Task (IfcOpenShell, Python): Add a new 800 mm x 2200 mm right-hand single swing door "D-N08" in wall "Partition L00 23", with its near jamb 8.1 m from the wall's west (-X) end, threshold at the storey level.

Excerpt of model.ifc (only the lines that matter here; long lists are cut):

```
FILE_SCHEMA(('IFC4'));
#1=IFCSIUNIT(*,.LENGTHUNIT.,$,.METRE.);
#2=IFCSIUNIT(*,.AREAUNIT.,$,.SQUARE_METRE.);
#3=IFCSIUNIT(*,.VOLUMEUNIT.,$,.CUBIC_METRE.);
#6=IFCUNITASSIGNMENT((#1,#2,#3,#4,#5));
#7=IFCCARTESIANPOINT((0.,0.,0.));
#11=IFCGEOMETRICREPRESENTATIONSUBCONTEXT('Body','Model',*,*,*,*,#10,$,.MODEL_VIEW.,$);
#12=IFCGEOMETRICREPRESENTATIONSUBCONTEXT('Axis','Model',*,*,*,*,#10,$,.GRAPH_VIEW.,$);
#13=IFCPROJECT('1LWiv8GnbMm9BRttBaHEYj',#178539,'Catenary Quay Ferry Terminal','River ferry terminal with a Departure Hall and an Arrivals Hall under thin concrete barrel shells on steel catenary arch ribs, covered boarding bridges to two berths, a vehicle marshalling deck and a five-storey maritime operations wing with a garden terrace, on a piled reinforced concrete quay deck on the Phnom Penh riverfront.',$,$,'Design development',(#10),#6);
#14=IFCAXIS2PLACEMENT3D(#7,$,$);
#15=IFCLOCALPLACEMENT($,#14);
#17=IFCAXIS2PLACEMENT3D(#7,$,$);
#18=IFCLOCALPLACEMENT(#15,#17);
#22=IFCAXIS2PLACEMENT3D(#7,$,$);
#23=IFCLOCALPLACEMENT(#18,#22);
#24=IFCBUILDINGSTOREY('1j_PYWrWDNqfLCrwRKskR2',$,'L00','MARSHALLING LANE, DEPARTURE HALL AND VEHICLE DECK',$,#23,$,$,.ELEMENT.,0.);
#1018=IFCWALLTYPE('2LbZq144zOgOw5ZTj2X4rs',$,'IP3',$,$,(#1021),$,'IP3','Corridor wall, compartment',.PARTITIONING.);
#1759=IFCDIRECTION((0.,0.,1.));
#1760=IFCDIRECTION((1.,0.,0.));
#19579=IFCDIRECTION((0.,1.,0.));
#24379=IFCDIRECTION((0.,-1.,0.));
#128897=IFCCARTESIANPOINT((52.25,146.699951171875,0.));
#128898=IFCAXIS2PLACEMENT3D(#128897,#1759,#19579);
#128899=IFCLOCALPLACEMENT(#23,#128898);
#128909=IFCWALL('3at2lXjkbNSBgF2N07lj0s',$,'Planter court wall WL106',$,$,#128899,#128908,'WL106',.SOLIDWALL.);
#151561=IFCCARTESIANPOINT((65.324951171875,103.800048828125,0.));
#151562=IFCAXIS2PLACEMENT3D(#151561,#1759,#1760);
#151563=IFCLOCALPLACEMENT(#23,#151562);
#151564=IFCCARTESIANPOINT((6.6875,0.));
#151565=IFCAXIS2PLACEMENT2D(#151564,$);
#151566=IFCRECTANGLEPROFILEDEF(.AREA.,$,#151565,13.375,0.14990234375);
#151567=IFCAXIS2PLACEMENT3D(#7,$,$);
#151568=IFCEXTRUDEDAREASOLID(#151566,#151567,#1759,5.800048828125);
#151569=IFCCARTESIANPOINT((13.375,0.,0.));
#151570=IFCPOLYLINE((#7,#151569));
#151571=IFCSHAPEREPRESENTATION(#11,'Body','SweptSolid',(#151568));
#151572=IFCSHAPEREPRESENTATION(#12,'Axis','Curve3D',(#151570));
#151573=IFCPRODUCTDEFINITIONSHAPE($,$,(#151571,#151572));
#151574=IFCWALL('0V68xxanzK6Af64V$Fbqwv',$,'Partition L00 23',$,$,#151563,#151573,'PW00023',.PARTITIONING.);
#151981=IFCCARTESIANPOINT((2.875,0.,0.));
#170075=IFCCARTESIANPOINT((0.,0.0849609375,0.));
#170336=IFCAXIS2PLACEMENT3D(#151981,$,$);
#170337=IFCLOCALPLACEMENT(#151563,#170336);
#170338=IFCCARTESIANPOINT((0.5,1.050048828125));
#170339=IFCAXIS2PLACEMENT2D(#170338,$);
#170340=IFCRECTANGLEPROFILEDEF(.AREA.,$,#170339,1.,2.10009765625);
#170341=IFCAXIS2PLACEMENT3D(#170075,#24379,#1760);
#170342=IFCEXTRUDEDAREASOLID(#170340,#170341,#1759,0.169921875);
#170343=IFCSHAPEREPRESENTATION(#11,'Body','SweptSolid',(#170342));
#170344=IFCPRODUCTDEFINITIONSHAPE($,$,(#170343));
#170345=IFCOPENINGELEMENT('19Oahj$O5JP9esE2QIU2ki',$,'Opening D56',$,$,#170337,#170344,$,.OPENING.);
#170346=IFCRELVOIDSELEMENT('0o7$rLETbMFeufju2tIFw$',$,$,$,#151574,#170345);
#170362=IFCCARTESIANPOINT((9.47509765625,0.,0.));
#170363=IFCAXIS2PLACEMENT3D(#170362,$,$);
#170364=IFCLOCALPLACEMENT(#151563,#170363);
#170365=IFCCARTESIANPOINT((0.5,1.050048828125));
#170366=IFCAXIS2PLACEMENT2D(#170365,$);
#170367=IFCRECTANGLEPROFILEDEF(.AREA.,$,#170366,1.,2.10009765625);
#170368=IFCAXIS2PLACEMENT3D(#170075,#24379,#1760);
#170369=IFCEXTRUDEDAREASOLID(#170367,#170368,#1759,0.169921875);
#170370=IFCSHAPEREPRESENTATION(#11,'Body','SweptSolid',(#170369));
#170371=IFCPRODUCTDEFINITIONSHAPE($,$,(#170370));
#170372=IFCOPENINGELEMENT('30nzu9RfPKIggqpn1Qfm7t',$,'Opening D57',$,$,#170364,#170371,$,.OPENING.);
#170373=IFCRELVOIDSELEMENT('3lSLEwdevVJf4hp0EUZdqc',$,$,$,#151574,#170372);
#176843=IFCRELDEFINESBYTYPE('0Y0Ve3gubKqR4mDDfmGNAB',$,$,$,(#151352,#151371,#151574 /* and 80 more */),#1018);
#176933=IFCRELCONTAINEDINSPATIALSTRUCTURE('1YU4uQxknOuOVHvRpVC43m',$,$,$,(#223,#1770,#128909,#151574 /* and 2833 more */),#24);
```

```python
import numpy as np
import ifcopenshell
import ifcopenshell.api.feature
import ifcopenshell.api.geometry
import ifcopenshell.api.root
import ifcopenshell.api.spatial
import ifcopenshell.geom
import ifcopenshell.util.element
import ifcopenshell.util.placement
import ifcopenshell.util.representation
import ifcopenshell.util.shape
import ifcopenshell.util.unit

model = ifcopenshell.open("model.ifc")
unit_scale = ifcopenshell.util.unit.calculate_unit_scale(model)
settings = ifcopenshell.geom.settings()


def volume(element):
    """Net volume in cubic metres, openings subtracted."""
    shape = ifcopenshell.geom.create_shape(settings, element)
    return ifcopenshell.util.shape.get_volume(shape.geometry)


wall = model.by_guid("0V68xxanzK6Af64V$Fbqwv")
storey = ifcopenshell.util.element.get_container(wall, ifc_class="IfcBuildingStorey")
context = ifcopenshell.util.representation.get_context(model, "Model", "Body", "MODEL_VIEW")
before = volume(wall)

width, height, from_end, sill = 0.8, 2.2, 8.1, 0.0  # metres

# The wall runs along its own X axis, and the end named is its -X end.
wall_shape = ifcopenshell.geom.create_shape(settings, wall)
x, y, z = ifcopenshell.util.shape.get_vertices(wall_shape.geometry).T
start = x.min() + from_end
face, thickness = float(y.min()), float(y.max() - y.min())
wall_matrix = ifcopenshell.util.placement.get_local_placement(wall.ObjectPlacement)
level = ifcopenshell.util.placement.get_local_placement(storey.ObjectPlacement)[2, 3]


def in_wall(x, y):
    """Placement at x, y metres in the wall's axes, at sill height."""
    matrix = wall_matrix.copy()
    matrix[:, 3] = wall_matrix @ np.array([x / unit_scale, y / unit_scale, 0.0, 1.0])
    matrix[2, 3] = level + sill / unit_scale
    return matrix


# Opening: a box that overshoots both wall faces by 50 mm.
opening = ifcopenshell.api.root.create_entity(model, ifc_class="IfcOpeningElement", predefined_type="OPENING")
box = ifcopenshell.api.geometry.add_wall_representation(
    model, context=context, length=width, height=height, thickness=thickness + 0.1
)
ifcopenshell.api.geometry.assign_representation(model, product=opening, representation=box)
ifcopenshell.api.geometry.edit_object_placement(model, product=opening, matrix=in_wall(start, face - 0.05), is_si=False)
ifcopenshell.api.feature.add_feature(model, feature=opening, element=wall)

door = ifcopenshell.api.root.create_entity(model, ifc_class="IfcDoor", name="D-N08", predefined_type="DOOR")
door.OverallWidth, door.OverallHeight = width / unit_scale, height / unit_scale
door.OperationType = "SINGLE_SWING_RIGHT"
body = ifcopenshell.api.geometry.add_door_representation(
    model,
    context=context,
    overall_width=door.OverallWidth,
    overall_height=door.OverallHeight,
    operation_type="SINGLE_SWING_RIGHT",
    lining_properties={"LiningDepth": thickness / unit_scale, "ThresholdDepth": thickness / unit_scale},
)
ifcopenshell.api.geometry.assign_representation(model, product=door, representation=body)
ifcopenshell.api.spatial.assign_container(model, products=[door], relating_structure=storey)
ifcopenshell.api.feature.add_filling(model, opening=opening, element=door)

# The lining spans the wall, so the door starts at the wall face.
ifcopenshell.api.geometry.edit_object_placement(model, product=door, matrix=in_wall(start, face), is_si=False)

after = volume(wall)

print(f"wall volume {before:.3f} -> {after:.3f} m3")

model.write("model_v2.ifc")
```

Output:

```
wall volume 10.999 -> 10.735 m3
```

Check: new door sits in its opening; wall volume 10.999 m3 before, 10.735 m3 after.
